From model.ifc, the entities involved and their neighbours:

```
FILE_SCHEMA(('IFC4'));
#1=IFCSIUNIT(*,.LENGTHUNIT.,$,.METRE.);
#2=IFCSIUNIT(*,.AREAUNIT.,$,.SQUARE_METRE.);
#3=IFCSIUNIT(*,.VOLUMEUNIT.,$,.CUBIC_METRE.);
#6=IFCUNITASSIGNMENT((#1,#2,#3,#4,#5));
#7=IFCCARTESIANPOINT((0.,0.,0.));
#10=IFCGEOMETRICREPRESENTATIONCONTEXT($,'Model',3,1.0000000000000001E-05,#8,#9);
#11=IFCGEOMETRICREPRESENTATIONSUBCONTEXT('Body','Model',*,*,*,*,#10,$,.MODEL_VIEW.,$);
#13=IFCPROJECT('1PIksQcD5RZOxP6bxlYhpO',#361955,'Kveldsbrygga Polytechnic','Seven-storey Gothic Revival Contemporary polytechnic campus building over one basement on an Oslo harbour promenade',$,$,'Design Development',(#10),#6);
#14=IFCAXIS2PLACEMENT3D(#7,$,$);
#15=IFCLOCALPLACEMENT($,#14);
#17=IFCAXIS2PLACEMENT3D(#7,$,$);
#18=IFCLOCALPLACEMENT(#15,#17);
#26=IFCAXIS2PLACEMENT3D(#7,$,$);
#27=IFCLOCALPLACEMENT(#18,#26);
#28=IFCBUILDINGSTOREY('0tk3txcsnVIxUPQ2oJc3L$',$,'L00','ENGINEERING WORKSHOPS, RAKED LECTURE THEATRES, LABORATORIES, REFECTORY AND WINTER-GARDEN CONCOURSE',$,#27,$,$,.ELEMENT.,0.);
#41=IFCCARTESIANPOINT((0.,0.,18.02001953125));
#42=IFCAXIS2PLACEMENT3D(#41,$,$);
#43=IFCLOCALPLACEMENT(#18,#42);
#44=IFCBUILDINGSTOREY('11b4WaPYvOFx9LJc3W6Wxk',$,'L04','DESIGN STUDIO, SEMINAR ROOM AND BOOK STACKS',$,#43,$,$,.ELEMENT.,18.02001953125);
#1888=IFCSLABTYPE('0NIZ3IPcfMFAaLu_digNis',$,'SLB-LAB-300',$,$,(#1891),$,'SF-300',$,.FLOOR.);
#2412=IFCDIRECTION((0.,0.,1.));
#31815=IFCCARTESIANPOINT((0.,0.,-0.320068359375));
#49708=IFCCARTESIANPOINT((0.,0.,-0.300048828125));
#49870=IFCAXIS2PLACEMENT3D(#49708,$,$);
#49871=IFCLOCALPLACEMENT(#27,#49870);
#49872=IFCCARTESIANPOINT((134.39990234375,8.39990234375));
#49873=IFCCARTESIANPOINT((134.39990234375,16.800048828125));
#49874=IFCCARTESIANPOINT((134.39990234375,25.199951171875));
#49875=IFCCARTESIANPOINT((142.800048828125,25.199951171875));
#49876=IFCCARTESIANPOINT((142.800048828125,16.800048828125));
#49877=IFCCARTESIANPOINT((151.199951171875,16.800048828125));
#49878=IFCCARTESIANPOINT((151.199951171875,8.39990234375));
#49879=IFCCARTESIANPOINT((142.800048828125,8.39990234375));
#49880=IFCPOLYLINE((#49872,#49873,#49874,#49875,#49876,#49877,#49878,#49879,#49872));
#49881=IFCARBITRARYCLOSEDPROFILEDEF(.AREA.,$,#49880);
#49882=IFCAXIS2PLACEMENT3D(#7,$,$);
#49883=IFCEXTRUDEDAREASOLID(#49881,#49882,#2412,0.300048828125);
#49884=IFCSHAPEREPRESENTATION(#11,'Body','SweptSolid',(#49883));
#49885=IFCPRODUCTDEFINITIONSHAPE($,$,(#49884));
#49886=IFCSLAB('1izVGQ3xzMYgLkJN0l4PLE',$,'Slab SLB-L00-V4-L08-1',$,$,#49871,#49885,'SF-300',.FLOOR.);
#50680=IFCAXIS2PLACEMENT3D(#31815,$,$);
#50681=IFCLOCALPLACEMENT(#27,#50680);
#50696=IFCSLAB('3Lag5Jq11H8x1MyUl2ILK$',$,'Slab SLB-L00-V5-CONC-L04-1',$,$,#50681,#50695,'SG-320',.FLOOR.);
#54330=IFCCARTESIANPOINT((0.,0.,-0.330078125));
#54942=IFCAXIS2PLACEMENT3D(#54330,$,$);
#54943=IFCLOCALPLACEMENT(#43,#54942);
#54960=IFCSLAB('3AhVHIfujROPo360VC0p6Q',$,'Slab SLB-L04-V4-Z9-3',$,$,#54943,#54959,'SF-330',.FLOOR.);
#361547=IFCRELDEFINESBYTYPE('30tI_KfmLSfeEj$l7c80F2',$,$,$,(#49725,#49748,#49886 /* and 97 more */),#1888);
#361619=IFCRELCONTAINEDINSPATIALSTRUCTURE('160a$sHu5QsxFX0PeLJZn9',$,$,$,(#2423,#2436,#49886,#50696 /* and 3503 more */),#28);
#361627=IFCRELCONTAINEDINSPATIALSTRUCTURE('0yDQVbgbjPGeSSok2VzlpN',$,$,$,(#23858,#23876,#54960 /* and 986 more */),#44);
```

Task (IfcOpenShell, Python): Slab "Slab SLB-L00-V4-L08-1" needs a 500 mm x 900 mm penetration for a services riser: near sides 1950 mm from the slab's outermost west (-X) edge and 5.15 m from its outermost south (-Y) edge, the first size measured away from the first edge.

```python
import numpy as np
import ifcopenshell
import ifcopenshell.api.feature
import ifcopenshell.api.geometry
import ifcopenshell.api.root
import ifcopenshell.geom
import ifcopenshell.util.placement
import ifcopenshell.util.representation
import ifcopenshell.util.shape
import ifcopenshell.util.unit

model = ifcopenshell.open("model.ifc")
unit_scale = ifcopenshell.util.unit.calculate_unit_scale(model)
settings = ifcopenshell.geom.settings()


def volume(element):
    """Net volume in cubic metres, openings subtracted."""
    shape = ifcopenshell.geom.create_shape(settings, element)
    return ifcopenshell.util.shape.get_volume(shape.geometry)


slab = model.by_guid("1izVGQ3xzMYgLkJN0l4PLE")
before = volume(slab)

# Extent in the slab's own axes, in metres. The edges named are its -X and -Y sides.
slab_shape = ifcopenshell.geom.create_shape(settings, slab)
vertices = ifcopenshell.util.shape.get_vertices(slab_shape.geometry)
x_min, y_min, bottom = vertices.min(axis=0)
top = vertices[:, 2].max()

opening = ifcopenshell.api.root.create_entity(model, ifc_class="IfcOpeningElement", name="Services riser opening", predefined_type="OPENING")
context = ifcopenshell.util.representation.get_context(model, "Model", "Body", "MODEL_VIEW")
width, depth = 0.5, 0.9
outline = [(0.0, 0.0), (width, 0.0), (width, depth), (0.0, depth), (0.0, 0.0)]
# Overshoot both faces by 50 mm so the cut is clean.
shape = ifcopenshell.api.geometry.add_slab_representation(
    model, context=context, depth=top - bottom + 0.1, polyline=outline
)
ifcopenshell.api.geometry.assign_representation(model, product=opening, representation=shape)

matrix = ifcopenshell.util.placement.get_local_placement(slab.ObjectPlacement)
matrix[:, 3] = matrix @ np.append(np.array([x_min + 1.95, y_min + 5.15, bottom - 0.05]) / unit_scale, 1.0)
ifcopenshell.api.geometry.edit_object_placement(model, product=opening, matrix=matrix, is_si=False)
ifcopenshell.api.feature.add_feature(model, feature=opening, element=slab)

after = volume(slab)

print(f"slab volume {before:.3f} -> {after:.3f} m3")

model.write("model_rev.ifc")
```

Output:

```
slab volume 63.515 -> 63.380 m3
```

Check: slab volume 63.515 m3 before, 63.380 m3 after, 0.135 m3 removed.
